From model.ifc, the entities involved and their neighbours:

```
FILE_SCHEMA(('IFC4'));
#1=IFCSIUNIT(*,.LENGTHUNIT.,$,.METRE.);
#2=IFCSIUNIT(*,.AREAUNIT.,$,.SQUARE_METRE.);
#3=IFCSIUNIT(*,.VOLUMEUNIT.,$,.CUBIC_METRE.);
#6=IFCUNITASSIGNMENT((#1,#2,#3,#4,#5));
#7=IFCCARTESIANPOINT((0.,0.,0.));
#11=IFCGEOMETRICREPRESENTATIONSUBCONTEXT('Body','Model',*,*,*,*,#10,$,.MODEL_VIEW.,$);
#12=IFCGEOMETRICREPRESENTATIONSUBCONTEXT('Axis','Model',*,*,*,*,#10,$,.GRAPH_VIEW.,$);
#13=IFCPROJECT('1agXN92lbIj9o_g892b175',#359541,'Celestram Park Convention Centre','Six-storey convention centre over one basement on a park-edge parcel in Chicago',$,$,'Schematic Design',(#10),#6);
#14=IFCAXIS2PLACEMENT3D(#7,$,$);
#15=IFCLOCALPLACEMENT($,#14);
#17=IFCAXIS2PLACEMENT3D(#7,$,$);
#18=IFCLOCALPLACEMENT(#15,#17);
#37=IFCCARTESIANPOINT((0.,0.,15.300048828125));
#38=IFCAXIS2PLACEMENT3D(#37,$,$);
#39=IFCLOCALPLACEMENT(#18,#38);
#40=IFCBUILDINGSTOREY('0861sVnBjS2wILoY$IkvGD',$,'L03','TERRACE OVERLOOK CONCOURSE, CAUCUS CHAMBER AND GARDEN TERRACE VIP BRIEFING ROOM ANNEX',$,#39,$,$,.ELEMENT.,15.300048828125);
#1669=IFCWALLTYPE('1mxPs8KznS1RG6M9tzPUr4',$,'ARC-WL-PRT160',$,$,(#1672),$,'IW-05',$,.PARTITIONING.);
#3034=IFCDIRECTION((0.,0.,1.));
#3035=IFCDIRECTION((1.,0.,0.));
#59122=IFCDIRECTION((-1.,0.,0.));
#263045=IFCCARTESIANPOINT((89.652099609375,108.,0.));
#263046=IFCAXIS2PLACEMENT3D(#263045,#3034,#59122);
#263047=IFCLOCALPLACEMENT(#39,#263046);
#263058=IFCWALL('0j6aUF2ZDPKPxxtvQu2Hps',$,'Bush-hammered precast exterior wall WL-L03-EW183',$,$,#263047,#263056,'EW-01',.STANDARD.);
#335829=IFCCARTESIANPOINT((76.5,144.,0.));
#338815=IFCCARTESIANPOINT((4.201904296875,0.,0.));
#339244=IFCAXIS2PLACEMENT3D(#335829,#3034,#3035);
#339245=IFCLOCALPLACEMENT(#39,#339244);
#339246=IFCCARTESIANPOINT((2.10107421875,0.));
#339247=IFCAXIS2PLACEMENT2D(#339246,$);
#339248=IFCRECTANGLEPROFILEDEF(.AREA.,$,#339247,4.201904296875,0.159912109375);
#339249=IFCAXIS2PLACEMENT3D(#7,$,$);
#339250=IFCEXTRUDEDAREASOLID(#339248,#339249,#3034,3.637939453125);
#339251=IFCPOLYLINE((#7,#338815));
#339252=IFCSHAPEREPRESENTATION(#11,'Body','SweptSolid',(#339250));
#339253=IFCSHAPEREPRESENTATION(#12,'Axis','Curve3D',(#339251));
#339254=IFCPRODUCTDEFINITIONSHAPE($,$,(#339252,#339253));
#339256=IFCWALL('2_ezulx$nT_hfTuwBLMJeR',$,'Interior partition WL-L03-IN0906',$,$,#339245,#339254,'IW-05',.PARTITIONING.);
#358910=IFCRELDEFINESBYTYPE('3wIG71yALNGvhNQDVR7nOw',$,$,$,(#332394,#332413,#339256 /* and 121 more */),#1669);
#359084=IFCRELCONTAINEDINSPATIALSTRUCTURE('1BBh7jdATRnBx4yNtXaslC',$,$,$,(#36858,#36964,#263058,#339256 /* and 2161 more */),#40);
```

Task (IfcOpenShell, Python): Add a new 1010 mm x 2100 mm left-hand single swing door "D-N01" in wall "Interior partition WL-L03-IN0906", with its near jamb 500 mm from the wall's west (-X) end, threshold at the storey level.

```python
import numpy as np
import ifcopenshell
import ifcopenshell.api.feature
import ifcopenshell.api.geometry
import ifcopenshell.api.root
import ifcopenshell.api.spatial
import ifcopenshell.geom
import ifcopenshell.util.element
import ifcopenshell.util.placement
import ifcopenshell.util.representation
import ifcopenshell.util.shape
import ifcopenshell.util.unit

model = ifcopenshell.open("model.ifc")
unit_scale = ifcopenshell.util.unit.calculate_unit_scale(model)
settings = ifcopenshell.geom.settings()


def volume(element):
    """Net volume in cubic metres, openings subtracted."""
    shape = ifcopenshell.geom.create_shape(settings, element)
    return ifcopenshell.util.shape.get_volume(shape.geometry)


wall = model.by_guid("2_ezulx$nT_hfTuwBLMJeR")
storey = ifcopenshell.util.element.get_container(wall, ifc_class="IfcBuildingStorey")
context = ifcopenshell.util.representation.get_context(model, "Model", "Body", "MODEL_VIEW")
before = volume(wall)

width, height, from_end, sill = 1.01, 2.1, 0.5, 0.0  # metres

# The wall runs along its own X axis, and the end named is its -X end.
wall_shape = ifcopenshell.geom.create_shape(settings, wall)
x, y, z = ifcopenshell.util.shape.get_vertices(wall_shape.geometry).T
start = x.min() + from_end
face, thickness = float(y.min()), float(y.max() - y.min())
wall_matrix = ifcopenshell.util.placement.get_local_placement(wall.ObjectPlacement)
level = ifcopenshell.util.placement.get_local_placement(storey.ObjectPlacement)[2, 3]


def in_wall(x, y):
    """Placement at x, y metres in the wall's axes, at sill height."""
    matrix = wall_matrix.copy()
    matrix[:, 3] = wall_matrix @ np.array([x / unit_scale, y / unit_scale, 0.0, 1.0])
    matrix[2, 3] = level + sill / unit_scale
    return matrix


# Opening: a box that overshoots both wall faces by 50 mm.
opening = ifcopenshell.api.root.create_entity(model, ifc_class="IfcOpeningElement", predefined_type="OPENING")
box = ifcopenshell.api.geometry.add_wall_representation(
    model, context=context, length=width, height=height, thickness=thickness + 0.1
)
ifcopenshell.api.geometry.assign_representation(model, product=opening, representation=box)
ifcopenshell.api.geometry.edit_object_placement(model, product=opening, matrix=in_wall(start, face - 0.05), is_si=False)
ifcopenshell.api.feature.add_feature(model, feature=opening, element=wall)

door = ifcopenshell.api.root.create_entity(model, ifc_class="IfcDoor", name="D-N01", predefined_type="DOOR")
door.OverallWidth, door.OverallHeight = width / unit_scale, height / unit_scale
door.OperationType = "SINGLE_SWING_LEFT"
body = ifcopenshell.api.geometry.add_door_representation(
    model,
    context=context,
    overall_width=door.OverallWidth,
    overall_height=door.OverallHeight,
    operation_type="SINGLE_SWING_LEFT",
    lining_properties={"LiningDepth": thickness / unit_scale, "ThresholdDepth": thickness / unit_scale},
)
ifcopenshell.api.geometry.assign_representation(model, product=door, representation=body)
ifcopenshell.api.spatial.assign_container(model, products=[door], relating_structure=storey)
ifcopenshell.api.feature.add_filling(model, opening=opening, element=door)

# The lining spans the wall, so the door starts at the wall face.
ifcopenshell.api.geometry.edit_object_placement(model, product=door, matrix=in_wall(start, face), is_si=False)

after = volume(wall)

print(f"wall volume {before:.3f} -> {after:.3f} m3")

model.write("model_rev.ifc")
```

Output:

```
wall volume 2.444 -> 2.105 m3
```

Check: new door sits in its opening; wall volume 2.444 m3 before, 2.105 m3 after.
